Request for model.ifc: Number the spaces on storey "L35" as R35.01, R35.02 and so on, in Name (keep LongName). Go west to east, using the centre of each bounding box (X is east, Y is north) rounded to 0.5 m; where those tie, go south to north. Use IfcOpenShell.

First a look at what the model holds.

```python
import ifcopenshell
import ifcopenshell.util.element
import ifcopenshell.util.placement

model = ifcopenshell.open("model.ifc")
print(model.schema)
storey = next(s for s in model.by_type("IfcBuildingStorey") if s.Name == "L35")
spaces = [e for e in ifcopenshell.util.element.get_decomposition(storey) if e.is_a("IfcSpace")]
for e in sorted(spaces, key=lambda e: e.id()):
    origin = ifcopenshell.util.placement.get_local_placement(e.ObjectPlacement)[:3, 3]
    print(e.id(), e.Name, e.LongName, origin.round(2) + 0.0, sep=" | ")
```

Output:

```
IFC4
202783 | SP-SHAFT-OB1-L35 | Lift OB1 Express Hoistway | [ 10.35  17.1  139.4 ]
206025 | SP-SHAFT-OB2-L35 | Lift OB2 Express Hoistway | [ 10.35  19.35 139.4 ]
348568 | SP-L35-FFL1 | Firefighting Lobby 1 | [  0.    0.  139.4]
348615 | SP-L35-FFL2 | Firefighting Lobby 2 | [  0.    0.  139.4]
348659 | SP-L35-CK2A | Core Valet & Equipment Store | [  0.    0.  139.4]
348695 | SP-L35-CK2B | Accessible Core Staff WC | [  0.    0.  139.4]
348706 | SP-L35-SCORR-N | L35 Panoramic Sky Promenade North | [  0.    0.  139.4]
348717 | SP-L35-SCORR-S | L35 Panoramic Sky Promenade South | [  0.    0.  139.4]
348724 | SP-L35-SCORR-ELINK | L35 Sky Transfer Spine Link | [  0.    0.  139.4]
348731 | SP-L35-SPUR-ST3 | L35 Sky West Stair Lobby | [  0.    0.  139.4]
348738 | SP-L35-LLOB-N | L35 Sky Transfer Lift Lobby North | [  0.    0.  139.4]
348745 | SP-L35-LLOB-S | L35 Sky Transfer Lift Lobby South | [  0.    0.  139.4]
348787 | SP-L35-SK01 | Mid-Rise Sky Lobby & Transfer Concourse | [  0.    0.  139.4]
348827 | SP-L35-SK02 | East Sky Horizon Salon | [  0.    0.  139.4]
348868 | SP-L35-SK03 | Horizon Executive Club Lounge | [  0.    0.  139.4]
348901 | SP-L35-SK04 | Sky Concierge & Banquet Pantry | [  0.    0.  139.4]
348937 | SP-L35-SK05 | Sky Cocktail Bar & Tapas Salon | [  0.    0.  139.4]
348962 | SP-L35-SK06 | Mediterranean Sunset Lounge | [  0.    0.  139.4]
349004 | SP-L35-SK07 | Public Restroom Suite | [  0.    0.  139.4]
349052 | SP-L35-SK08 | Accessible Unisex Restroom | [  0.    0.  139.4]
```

```python
import ifcopenshell
import ifcopenshell.geom
import ifcopenshell.util.element
import ifcopenshell.util.shape

model = ifcopenshell.open("model.ifc")
settings = ifcopenshell.geom.settings()
settings.set("use-world-coords", True)


def centre(element):
    shape = ifcopenshell.geom.create_shape(settings, element)
    return ifcopenshell.util.shape.get_bbox_centroid(shape.geometry)


storey = next(s for s in model.by_type("IfcBuildingStorey") if s.Name == "L35")
spaces = [e for e in ifcopenshell.util.element.get_decomposition(storey) if e.is_a("IfcSpace")]

# Insertion points can sit at a corner or the storey origin, so sort by the geometry (in metres).
centres = {e: centre(e) for e in spaces}
spaces.sort(key=lambda e: (round(centres[e][0] / 0.5), centres[e][1]))

for i, e in enumerate(spaces, start=1):
    number = f"R35.{i:02d}"
    e.Name = number
    print(e.id(), number)

model.write("model_v2.ifc")
```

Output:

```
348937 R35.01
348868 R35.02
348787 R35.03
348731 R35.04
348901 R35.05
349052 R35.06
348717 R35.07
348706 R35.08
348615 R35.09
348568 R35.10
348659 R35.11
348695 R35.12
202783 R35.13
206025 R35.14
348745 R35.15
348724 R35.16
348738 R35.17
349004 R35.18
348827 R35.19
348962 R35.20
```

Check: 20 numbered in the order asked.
